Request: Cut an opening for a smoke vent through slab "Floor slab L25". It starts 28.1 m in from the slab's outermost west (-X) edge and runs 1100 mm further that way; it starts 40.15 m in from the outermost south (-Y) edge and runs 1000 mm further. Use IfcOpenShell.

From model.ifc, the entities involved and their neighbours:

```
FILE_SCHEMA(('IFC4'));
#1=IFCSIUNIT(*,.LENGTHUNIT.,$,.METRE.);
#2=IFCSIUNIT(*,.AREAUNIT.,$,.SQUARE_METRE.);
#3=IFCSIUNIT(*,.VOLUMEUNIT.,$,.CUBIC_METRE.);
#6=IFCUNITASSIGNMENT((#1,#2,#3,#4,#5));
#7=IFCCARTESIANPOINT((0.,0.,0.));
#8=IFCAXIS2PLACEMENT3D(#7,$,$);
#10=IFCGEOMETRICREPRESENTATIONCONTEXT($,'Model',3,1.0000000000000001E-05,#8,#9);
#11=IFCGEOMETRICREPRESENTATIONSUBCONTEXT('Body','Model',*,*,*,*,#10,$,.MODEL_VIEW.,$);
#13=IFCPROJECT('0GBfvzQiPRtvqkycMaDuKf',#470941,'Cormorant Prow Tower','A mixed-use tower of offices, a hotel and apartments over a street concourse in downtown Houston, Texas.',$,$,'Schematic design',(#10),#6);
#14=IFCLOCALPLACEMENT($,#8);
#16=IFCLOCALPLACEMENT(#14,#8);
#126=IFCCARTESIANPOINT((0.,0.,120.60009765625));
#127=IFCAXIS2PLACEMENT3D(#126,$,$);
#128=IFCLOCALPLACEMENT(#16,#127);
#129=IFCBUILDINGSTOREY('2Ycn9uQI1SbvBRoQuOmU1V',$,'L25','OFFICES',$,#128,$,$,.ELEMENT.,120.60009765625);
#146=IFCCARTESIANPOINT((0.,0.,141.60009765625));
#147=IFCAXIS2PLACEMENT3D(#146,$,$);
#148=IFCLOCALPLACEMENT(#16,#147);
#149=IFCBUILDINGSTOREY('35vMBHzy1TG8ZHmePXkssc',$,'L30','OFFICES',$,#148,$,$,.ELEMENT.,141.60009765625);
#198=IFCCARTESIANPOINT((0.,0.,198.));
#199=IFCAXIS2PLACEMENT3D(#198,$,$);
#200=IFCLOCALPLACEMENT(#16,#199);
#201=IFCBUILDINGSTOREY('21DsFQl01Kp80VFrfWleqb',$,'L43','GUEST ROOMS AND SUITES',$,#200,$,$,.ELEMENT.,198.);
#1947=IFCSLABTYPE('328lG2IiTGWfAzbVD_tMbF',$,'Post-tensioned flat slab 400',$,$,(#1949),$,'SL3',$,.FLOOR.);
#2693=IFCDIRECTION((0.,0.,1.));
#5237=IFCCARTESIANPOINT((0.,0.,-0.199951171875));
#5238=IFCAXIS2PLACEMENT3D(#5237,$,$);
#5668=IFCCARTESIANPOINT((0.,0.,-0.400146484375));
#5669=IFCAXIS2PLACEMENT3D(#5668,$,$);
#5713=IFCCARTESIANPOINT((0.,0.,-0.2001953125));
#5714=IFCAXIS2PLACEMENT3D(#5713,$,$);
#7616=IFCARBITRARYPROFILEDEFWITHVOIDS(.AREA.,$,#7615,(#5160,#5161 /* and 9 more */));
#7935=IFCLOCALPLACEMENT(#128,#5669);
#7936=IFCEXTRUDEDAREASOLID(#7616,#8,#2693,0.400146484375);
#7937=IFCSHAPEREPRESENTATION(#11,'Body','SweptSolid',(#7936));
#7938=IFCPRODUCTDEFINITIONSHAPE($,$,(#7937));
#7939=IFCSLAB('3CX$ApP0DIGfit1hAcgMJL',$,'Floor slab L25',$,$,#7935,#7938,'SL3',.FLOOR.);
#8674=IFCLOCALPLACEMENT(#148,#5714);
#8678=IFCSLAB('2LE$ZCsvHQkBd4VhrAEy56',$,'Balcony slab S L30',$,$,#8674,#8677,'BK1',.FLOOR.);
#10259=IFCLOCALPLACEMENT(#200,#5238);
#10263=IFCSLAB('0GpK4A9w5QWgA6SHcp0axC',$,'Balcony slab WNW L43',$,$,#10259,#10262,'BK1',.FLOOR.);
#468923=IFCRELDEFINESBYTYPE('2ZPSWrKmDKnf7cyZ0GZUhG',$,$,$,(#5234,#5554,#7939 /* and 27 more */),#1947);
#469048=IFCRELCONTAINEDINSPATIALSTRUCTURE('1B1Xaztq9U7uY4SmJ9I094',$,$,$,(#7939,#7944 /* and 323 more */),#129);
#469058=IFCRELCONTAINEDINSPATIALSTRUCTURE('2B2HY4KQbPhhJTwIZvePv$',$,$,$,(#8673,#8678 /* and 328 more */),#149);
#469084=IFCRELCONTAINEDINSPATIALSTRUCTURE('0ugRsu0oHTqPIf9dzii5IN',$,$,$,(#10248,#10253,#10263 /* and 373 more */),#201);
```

```python
import numpy as np
import ifcopenshell
import ifcopenshell.api.feature
import ifcopenshell.api.geometry
import ifcopenshell.api.root
import ifcopenshell.geom
import ifcopenshell.util.placement
import ifcopenshell.util.representation
import ifcopenshell.util.shape
import ifcopenshell.util.unit

model = ifcopenshell.open("model.ifc")
unit_scale = ifcopenshell.util.unit.calculate_unit_scale(model)
settings = ifcopenshell.geom.settings()


def volume(element):
    """Net volume in cubic metres, openings subtracted."""
    shape = ifcopenshell.geom.create_shape(settings, element)
    return ifcopenshell.util.shape.get_volume(shape.geometry)


slab = model.by_id(7939)
before = volume(slab)

# Extent in the slab's own axes, in metres. The edges named are its -X and -Y sides.
slab_shape = ifcopenshell.geom.create_shape(settings, slab)
vertices = ifcopenshell.util.shape.get_vertices(slab_shape.geometry)
x_min, y_min, bottom = vertices.min(axis=0)
top = vertices[:, 2].max()

opening = ifcopenshell.api.root.create_entity(model, ifc_class="IfcOpeningElement", name="Smoke vent opening", predefined_type="OPENING")
context = ifcopenshell.util.representation.get_context(model, "Model", "Body", "MODEL_VIEW")
width, depth = 1.1, 1
outline = [(0.0, 0.0), (width, 0.0), (width, depth), (0.0, depth), (0.0, 0.0)]
# Overshoot both faces by 50 mm so the cut is clean.
shape = ifcopenshell.api.geometry.add_slab_representation(
    model, context=context, depth=top - bottom + 0.1, polyline=outline
)
ifcopenshell.api.geometry.assign_representation(model, product=opening, representation=shape)

matrix = ifcopenshell.util.placement.get_local_placement(slab.ObjectPlacement)
matrix[:, 3] = matrix @ np.append(np.array([x_min + 28.1, y_min + 40.15, bottom - 0.05]) / unit_scale, 1.0)
ifcopenshell.api.geometry.edit_object_placement(model, product=opening, matrix=matrix, is_si=False)
ifcopenshell.api.feature.add_feature(model, feature=opening, element=slab)

after = volume(slab)

print(f"slab volume {before:.3f} -> {after:.3f} m3")

model.write("model_rev.ifc")
```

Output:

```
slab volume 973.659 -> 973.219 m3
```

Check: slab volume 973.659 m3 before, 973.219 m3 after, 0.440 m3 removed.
